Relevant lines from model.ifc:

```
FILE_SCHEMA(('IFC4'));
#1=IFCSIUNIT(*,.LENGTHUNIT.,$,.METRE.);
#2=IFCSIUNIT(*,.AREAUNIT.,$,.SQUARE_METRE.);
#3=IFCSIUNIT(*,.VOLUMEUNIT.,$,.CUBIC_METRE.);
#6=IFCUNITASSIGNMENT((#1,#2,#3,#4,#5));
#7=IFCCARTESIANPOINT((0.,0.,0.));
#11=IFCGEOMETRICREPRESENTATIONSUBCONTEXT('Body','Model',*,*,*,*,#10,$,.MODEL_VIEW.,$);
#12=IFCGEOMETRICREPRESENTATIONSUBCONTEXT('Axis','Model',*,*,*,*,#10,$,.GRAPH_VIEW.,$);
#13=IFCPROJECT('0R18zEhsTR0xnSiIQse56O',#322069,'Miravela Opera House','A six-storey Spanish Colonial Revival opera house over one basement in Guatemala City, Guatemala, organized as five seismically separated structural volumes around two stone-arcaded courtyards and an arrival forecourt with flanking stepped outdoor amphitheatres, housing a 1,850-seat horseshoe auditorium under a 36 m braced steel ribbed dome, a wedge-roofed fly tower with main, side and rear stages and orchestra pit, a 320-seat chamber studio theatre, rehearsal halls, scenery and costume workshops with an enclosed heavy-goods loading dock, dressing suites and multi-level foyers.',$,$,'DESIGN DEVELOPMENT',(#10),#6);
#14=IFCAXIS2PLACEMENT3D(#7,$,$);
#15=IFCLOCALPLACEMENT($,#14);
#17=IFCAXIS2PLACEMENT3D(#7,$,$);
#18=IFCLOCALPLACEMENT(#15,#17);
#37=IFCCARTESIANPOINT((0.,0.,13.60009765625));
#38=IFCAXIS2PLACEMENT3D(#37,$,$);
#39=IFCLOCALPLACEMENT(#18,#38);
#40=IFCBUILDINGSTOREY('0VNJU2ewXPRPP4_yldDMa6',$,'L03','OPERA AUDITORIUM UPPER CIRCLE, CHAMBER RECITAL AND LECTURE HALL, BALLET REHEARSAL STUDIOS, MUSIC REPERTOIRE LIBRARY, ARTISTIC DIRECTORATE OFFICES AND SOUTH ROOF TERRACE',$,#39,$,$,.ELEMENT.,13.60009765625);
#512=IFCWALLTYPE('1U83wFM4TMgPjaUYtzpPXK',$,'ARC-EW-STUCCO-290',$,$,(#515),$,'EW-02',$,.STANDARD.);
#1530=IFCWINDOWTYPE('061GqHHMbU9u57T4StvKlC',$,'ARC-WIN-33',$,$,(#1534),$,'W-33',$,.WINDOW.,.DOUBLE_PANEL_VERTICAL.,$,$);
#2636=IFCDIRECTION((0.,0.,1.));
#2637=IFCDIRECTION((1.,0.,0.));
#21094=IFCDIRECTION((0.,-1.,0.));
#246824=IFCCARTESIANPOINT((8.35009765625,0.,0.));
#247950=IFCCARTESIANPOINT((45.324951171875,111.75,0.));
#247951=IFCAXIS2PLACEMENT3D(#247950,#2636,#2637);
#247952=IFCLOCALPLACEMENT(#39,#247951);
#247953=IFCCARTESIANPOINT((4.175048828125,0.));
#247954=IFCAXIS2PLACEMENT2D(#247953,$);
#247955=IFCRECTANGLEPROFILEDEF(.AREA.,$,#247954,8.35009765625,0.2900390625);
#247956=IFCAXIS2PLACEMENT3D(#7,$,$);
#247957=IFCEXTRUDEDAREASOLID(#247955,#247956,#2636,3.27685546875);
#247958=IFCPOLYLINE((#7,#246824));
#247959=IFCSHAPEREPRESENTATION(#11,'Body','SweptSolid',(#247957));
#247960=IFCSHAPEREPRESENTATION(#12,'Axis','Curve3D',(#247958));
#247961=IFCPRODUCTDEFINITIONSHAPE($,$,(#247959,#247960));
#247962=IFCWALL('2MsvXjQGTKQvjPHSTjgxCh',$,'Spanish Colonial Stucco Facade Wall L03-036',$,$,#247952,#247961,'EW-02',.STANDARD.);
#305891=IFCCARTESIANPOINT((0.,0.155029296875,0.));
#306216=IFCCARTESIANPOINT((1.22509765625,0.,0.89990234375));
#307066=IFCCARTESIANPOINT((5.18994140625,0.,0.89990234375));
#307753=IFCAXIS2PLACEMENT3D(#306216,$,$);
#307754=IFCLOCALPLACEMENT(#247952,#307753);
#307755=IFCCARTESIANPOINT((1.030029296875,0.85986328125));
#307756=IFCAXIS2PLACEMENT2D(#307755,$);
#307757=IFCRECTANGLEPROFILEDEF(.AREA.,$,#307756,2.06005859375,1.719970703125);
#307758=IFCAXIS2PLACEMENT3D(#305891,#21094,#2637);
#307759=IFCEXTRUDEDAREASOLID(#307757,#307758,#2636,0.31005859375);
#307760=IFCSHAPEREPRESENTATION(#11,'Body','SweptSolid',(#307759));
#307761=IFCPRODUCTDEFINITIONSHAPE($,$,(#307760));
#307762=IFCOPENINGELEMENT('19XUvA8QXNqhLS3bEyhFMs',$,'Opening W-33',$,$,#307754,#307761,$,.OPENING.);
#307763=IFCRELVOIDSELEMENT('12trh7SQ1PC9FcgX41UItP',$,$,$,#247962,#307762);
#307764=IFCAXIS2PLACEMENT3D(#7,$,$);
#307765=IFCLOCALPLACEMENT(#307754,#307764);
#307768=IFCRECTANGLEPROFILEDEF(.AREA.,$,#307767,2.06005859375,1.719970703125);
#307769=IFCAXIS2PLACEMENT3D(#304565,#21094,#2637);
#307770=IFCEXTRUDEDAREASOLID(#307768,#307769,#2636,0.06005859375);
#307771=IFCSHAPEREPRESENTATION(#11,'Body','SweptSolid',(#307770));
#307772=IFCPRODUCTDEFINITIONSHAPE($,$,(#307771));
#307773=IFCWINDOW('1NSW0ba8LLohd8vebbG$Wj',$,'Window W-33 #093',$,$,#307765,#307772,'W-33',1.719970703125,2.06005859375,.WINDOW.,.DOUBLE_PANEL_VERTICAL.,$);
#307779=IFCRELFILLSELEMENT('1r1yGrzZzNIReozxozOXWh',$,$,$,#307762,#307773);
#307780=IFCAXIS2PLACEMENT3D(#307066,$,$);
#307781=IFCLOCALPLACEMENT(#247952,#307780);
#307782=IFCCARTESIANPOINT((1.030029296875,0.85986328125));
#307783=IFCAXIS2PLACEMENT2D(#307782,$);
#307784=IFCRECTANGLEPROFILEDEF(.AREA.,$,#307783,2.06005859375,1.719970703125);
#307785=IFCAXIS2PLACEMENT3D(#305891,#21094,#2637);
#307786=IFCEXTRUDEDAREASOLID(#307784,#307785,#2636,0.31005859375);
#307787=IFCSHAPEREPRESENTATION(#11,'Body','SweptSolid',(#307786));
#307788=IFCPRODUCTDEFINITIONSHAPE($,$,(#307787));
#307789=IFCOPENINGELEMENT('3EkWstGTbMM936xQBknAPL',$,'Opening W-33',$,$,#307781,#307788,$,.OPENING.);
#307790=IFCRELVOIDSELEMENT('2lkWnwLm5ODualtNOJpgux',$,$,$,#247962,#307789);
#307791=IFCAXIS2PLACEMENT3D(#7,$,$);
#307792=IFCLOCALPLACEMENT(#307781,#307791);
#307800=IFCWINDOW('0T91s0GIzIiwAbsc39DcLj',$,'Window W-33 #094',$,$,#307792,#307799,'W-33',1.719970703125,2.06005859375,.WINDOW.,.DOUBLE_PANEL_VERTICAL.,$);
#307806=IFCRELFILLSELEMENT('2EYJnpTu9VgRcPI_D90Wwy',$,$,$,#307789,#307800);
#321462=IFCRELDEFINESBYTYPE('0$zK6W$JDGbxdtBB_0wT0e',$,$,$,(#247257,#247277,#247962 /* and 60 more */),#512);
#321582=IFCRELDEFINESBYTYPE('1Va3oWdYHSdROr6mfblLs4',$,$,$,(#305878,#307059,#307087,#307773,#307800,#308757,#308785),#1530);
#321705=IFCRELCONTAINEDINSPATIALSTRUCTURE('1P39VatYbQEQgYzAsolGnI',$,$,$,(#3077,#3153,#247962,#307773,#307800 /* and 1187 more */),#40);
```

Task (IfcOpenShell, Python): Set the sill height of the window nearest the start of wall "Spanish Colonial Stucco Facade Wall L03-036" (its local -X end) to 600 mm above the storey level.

```python
import numpy as np
import ifcopenshell
import ifcopenshell.api.geometry
import ifcopenshell.geom
import ifcopenshell.util.element
import ifcopenshell.util.placement
import ifcopenshell.util.shape
import ifcopenshell.util.unit

model = ifcopenshell.open("model.ifc")
unit_scale = ifcopenshell.util.unit.calculate_unit_scale(model)

window = model.by_guid("1NSW0ba8LLohd8vebbG$Wj")
opening = window.FillsVoids[0].RelatingOpeningElement
storey = ifcopenshell.util.element.get_container(window, ifc_class="IfcBuildingStorey")
level = ifcopenshell.util.placement.get_local_placement(storey.ObjectPlacement)[2, 3]

# The opening's origin need not be at the sill, so measure its lowest point.
shape = ifcopenshell.geom.create_shape(ifcopenshell.geom.settings(), opening)
bottom = ifcopenshell.util.shape.get_shape_bottom_elevation(shape, shape.geometry) / unit_scale
dz = level + 0.6 / unit_scale - bottom

shift = np.array([0.0, 0.0, dz])
# The window is placed relative to its opening, so it follows when the opening moves.
matrix = ifcopenshell.util.placement.get_local_placement(opening.ObjectPlacement)
matrix[:3, 3] += shift
ifcopenshell.api.geometry.edit_object_placement(
    model, product=opening, matrix=matrix, is_si=False, should_transform_children=True
)

print(f"moved by {dz * unit_scale:+.3f} m")

model.write("model_updated.ifc")
```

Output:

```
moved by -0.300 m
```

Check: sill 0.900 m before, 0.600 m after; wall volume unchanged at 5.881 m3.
